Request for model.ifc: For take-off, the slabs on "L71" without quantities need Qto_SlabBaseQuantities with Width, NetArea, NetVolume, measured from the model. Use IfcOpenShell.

First a look at what the model holds.

```python
import ifcopenshell
import ifcopenshell.util.element
import ifcopenshell.util.unit

model = ifcopenshell.open("model.ifc")
print(model.schema)
for unit_type in ("LENGTHUNIT", "AREAUNIT", "VOLUMEUNIT"):
    print(unit_type, ifcopenshell.util.unit.calculate_unit_scale(model, unit_type))
storey = next(s for s in model.by_type("IfcBuildingStorey") if s.Name == "L71")
slabs = [e for e in ifcopenshell.util.element.get_decomposition(storey) if e.is_a("IfcSlab")]
for e in sorted(slabs, key=lambda e: e.id()):
    print(e.id(), e.is_a(), e.Name, list(ifcopenshell.util.element.get_psets(e, qtos_only=True)), sep=" | ")
```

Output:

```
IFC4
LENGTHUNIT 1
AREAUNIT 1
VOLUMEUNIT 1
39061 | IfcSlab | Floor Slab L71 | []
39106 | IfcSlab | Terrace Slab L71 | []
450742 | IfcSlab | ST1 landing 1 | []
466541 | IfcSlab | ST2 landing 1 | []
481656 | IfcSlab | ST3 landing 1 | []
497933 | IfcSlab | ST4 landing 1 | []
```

```python
import ifcopenshell
import ifcopenshell.api.pset
import ifcopenshell.geom
import ifcopenshell.util.element
import ifcopenshell.util.shape
import ifcopenshell.util.unit

model = ifcopenshell.open("model.ifc")
unit_scale = ifcopenshell.util.unit.calculate_unit_scale(model)
area_scale = ifcopenshell.util.unit.calculate_unit_scale(model, "AREAUNIT")
volume_scale = ifcopenshell.util.unit.calculate_unit_scale(model, "VOLUMEUNIT")
settings = ifcopenshell.geom.settings()

storey = next(s for s in model.by_type("IfcBuildingStorey") if s.Name == "L71")
slabs = [e for e in ifcopenshell.util.element.get_decomposition(storey) if e.is_a("IfcSlab")]

for e in sorted(slabs, key=lambda e: e.id()):
    if ifcopenshell.util.element.get_psets(e, qtos_only=True, should_inherit=False):
        continue
    # Geometry comes back in metres, in the element's own axes.
    shape = ifcopenshell.geom.create_shape(settings, e)
    values = {
        "Width": ifcopenshell.util.shape.get_z(shape.geometry) / unit_scale,
        "NetArea": ifcopenshell.util.shape.get_footprint_area(shape.geometry) / area_scale,
        "NetVolume": ifcopenshell.util.shape.get_volume(shape.geometry) / volume_scale,
    }
    qto = ifcopenshell.api.pset.add_qto(model, product=e, name="Qto_SlabBaseQuantities")
    ifcopenshell.api.pset.edit_qto(model, qto=qto, properties=values)
    print(e.id(), {k: round(v, 3) for k, v in values.items()})

model.write("model_rev.ifc")
```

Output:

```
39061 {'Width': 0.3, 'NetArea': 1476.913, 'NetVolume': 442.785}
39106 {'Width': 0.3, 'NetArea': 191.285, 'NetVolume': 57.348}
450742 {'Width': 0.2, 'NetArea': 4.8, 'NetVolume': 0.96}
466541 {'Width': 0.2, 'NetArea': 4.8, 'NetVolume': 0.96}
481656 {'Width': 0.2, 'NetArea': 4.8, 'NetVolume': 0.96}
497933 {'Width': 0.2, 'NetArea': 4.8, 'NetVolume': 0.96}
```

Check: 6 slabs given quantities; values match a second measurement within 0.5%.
